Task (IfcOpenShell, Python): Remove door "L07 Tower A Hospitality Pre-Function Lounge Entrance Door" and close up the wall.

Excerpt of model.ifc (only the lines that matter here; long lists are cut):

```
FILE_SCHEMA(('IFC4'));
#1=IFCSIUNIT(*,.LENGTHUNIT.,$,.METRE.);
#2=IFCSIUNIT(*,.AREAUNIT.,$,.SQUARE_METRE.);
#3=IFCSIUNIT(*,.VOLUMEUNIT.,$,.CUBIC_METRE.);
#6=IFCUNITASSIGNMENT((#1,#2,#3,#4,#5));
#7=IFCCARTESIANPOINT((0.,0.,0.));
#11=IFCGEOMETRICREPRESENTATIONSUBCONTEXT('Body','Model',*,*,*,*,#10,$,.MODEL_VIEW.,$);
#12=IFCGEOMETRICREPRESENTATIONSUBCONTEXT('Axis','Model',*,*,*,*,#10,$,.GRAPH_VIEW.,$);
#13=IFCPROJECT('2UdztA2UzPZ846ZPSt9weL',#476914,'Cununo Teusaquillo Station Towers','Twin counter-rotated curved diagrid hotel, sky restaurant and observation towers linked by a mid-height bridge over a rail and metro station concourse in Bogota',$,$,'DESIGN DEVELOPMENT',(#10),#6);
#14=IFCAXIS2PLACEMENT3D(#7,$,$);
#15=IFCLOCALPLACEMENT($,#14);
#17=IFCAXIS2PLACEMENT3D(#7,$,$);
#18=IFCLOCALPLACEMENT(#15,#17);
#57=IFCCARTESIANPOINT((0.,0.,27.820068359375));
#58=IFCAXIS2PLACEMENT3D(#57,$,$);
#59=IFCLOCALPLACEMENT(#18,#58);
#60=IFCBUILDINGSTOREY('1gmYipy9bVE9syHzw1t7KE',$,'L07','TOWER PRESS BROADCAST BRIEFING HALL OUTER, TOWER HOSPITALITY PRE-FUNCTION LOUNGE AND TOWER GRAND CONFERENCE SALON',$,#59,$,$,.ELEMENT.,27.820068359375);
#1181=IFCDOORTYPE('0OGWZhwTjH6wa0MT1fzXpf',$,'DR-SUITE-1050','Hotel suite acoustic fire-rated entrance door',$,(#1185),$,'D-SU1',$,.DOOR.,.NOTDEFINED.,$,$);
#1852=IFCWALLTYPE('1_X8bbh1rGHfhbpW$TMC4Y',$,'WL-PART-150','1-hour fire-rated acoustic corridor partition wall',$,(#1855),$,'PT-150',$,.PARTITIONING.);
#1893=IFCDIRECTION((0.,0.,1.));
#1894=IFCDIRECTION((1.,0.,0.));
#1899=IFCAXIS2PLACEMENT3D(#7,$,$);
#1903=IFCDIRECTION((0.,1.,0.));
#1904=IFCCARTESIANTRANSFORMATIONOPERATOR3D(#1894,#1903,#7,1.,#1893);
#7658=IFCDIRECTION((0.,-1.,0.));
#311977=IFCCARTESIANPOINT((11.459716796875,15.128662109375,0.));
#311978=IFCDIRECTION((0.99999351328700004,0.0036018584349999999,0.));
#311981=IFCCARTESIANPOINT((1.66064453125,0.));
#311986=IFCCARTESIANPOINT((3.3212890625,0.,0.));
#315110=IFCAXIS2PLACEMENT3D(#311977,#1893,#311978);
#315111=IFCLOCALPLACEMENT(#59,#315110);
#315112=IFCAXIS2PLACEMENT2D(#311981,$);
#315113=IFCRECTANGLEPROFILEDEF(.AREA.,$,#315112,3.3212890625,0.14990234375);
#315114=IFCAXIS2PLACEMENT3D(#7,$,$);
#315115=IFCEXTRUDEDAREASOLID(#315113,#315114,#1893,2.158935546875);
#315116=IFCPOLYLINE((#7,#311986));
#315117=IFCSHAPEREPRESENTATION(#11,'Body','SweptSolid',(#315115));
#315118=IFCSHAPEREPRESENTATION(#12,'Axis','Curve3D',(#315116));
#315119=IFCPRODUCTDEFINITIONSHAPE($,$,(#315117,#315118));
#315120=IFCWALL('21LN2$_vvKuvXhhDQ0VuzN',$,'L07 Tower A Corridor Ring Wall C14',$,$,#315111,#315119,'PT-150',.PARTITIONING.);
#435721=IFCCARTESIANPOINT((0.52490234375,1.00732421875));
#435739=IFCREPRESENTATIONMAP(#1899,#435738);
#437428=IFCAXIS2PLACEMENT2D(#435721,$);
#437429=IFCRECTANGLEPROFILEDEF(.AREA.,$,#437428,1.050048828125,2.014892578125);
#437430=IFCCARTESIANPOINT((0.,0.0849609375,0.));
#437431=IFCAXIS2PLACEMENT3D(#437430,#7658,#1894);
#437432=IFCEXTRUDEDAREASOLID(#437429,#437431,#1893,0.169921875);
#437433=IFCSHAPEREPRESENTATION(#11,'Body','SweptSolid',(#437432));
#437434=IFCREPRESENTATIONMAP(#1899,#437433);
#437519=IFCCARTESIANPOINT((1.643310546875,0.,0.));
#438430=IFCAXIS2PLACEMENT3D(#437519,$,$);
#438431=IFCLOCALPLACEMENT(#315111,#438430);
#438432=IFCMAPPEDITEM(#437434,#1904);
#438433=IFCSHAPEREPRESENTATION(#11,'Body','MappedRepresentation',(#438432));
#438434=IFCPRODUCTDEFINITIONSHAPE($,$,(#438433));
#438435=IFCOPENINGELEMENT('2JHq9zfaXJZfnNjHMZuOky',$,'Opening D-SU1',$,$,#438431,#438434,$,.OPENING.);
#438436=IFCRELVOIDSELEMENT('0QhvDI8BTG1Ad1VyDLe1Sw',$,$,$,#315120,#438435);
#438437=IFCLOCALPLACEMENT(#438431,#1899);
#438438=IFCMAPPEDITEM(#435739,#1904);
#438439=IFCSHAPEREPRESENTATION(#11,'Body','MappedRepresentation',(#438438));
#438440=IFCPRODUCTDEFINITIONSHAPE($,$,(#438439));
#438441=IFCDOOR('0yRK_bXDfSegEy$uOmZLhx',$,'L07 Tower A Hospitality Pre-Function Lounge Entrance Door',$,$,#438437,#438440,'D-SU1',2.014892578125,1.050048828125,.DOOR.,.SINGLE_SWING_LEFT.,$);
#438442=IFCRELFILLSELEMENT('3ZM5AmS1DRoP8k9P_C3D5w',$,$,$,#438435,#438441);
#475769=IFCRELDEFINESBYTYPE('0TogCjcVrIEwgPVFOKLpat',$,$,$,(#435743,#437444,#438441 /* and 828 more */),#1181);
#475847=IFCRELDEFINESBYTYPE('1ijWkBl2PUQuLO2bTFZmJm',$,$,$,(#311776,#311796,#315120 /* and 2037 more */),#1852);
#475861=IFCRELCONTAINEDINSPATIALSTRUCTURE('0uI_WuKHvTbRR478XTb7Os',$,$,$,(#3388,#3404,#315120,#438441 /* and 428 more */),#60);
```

```python
import ifcopenshell
import ifcopenshell.api.feature
import ifcopenshell.api.root
import ifcopenshell.geom
import ifcopenshell.util.shape

model = ifcopenshell.open("model.ifc")
settings = ifcopenshell.geom.settings()


def volume(element):
    """Net volume in cubic metres, openings subtracted."""
    shape = ifcopenshell.geom.create_shape(settings, element)
    return ifcopenshell.util.shape.get_volume(shape.geometry)


door = model.by_guid("0yRK_bXDfSegEy$uOmZLhx")
opening = door.FillsVoids[0].RelatingOpeningElement
wall = opening.VoidsElements[0].RelatingBuildingElement
before = volume(wall)

ifcopenshell.api.root.remove_product(model, product=door)
ifcopenshell.api.feature.remove_feature(model, feature=opening)

after = volume(wall)

print(f"wall volume {before:.3f} -> {after:.3f} m3")

model.write("model_updated.ifc")
```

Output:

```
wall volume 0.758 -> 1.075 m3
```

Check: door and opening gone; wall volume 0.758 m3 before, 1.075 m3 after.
